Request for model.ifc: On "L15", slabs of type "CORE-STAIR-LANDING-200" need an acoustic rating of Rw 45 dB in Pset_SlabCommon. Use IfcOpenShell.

First a look at what the model holds.

```python
import ifcopenshell
import ifcopenshell.util.element

model = ifcopenshell.open("model.ifc")
print(model.schema)
storey = next(s for s in model.by_type("IfcBuildingStorey") if s.Name == "L15")
slabs = [e for e in ifcopenshell.util.element.get_decomposition(storey) if e.is_a("IfcSlab")]
seen = {}
for e in slabs:
    element_type = ifcopenshell.util.element.get_type(e)
    key = (element_type.Name if element_type != e and element_type else None, ifcopenshell.util.element.get_pset(e, "Pset_SlabCommon", "AcousticRating"))
    seen[key] = seen.get(key, 0) + 1
for (name, value), count in sorted(seen.items(), key=str):
    print(count, "x", name, "|", value)
```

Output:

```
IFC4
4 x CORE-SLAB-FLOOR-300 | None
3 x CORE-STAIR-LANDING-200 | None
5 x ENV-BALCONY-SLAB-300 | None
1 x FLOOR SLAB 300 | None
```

```python
import ifcopenshell
import ifcopenshell.api.pset
import ifcopenshell.util.element

model = ifcopenshell.open("model.ifc")

storey = next(s for s in model.by_type("IfcBuildingStorey") if s.Name == "L15")
slabs = [e for e in ifcopenshell.util.element.get_decomposition(storey) if e.is_a("IfcSlab")]

count = 0
for e in slabs:
    element_type = ifcopenshell.util.element.get_type(e)
    if element_type in (None, e) or element_type.Name != "CORE-STAIR-LANDING-200":
        continue
    found = ifcopenshell.util.element.get_pset(e, "Pset_SlabCommon", should_inherit=False)
    if found:
        pset = model.by_id(found["id"])
        if len(ifcopenshell.util.element.get_elements_by_pset(pset)) > 1:
            pset = ifcopenshell.api.pset.unshare_pset(model, products=[e], pset=pset)[0]
    else:
        pset = ifcopenshell.api.pset.add_pset(model, product=e, name="Pset_SlabCommon")
    ifcopenshell.api.pset.edit_pset(model, pset=pset, properties={"AcousticRating": "Rw 45 dB"})
    count += 1

print(count, "slabs updated")

model.write("model_edited.ifc")
```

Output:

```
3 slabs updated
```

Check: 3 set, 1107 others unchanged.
